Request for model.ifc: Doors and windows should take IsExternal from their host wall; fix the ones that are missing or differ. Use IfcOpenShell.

First a look at what the model holds.

```python
import ifcopenshell
import ifcopenshell.util.element

model = ifcopenshell.open("model.ifc")
print(model.schema)
seen = {}
for e in model.by_type("IfcDoor") + model.by_type("IfcWindow"):
    if not e.FillsVoids:
        continue
    host = e.FillsVoids[0].RelatingOpeningElement.VoidsElements[0].RelatingBuildingElement
    own = ifcopenshell.util.element.get_pset(e, f"Pset_{e.is_a()[3:].removesuffix('StandardCase')}Common", "IsExternal")
    wall = ifcopenshell.util.element.get_pset(host, "Pset_WallCommon", "IsExternal")
    seen[e.is_a(), own, wall] = seen.get((e.is_a(), own, wall), 0) + 1
for (cls, own, wall), count in sorted(seen.items(), key=str):
    print(count, cls, "IsExternal:", own, "| host wall:", wall)
```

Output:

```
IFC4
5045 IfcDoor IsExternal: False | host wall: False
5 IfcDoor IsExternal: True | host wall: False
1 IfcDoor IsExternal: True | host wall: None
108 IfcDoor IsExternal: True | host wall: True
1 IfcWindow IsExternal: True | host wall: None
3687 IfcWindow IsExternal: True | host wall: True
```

```python
import ifcopenshell
import ifcopenshell.api.pset
import ifcopenshell.util.element

model = ifcopenshell.open("model.ifc")

count = 0
for ifc_class, pset_name in (("IfcDoor", "Pset_DoorCommon"), ("IfcWindow", "Pset_WindowCommon")):
    for e in model.by_type(ifc_class):
        if not e.FillsVoids:
            continue
        host = e.FillsVoids[0].RelatingOpeningElement.VoidsElements[0].RelatingBuildingElement
        external = ifcopenshell.util.element.get_pset(host, "Pset_WallCommon", "IsExternal")
        if external is None or ifcopenshell.util.element.get_pset(e, pset_name, "IsExternal") == external:
            continue
        found = ifcopenshell.util.element.get_pset(e, pset_name, should_inherit=False)
        if found:
            pset = model.by_id(found["id"])
            if len(ifcopenshell.util.element.get_elements_by_pset(pset)) > 1:
                pset = ifcopenshell.api.pset.unshare_pset(model, products=[e], pset=pset)[0]
        else:
            pset = ifcopenshell.api.pset.add_pset(model, product=e, name=pset_name)
        ifcopenshell.api.pset.edit_pset(model, pset=pset, properties={"IsExternal": external})
        count += 1

print(count, "updated")

model.write("model_rev.ifc")
```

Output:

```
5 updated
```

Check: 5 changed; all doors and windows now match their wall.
